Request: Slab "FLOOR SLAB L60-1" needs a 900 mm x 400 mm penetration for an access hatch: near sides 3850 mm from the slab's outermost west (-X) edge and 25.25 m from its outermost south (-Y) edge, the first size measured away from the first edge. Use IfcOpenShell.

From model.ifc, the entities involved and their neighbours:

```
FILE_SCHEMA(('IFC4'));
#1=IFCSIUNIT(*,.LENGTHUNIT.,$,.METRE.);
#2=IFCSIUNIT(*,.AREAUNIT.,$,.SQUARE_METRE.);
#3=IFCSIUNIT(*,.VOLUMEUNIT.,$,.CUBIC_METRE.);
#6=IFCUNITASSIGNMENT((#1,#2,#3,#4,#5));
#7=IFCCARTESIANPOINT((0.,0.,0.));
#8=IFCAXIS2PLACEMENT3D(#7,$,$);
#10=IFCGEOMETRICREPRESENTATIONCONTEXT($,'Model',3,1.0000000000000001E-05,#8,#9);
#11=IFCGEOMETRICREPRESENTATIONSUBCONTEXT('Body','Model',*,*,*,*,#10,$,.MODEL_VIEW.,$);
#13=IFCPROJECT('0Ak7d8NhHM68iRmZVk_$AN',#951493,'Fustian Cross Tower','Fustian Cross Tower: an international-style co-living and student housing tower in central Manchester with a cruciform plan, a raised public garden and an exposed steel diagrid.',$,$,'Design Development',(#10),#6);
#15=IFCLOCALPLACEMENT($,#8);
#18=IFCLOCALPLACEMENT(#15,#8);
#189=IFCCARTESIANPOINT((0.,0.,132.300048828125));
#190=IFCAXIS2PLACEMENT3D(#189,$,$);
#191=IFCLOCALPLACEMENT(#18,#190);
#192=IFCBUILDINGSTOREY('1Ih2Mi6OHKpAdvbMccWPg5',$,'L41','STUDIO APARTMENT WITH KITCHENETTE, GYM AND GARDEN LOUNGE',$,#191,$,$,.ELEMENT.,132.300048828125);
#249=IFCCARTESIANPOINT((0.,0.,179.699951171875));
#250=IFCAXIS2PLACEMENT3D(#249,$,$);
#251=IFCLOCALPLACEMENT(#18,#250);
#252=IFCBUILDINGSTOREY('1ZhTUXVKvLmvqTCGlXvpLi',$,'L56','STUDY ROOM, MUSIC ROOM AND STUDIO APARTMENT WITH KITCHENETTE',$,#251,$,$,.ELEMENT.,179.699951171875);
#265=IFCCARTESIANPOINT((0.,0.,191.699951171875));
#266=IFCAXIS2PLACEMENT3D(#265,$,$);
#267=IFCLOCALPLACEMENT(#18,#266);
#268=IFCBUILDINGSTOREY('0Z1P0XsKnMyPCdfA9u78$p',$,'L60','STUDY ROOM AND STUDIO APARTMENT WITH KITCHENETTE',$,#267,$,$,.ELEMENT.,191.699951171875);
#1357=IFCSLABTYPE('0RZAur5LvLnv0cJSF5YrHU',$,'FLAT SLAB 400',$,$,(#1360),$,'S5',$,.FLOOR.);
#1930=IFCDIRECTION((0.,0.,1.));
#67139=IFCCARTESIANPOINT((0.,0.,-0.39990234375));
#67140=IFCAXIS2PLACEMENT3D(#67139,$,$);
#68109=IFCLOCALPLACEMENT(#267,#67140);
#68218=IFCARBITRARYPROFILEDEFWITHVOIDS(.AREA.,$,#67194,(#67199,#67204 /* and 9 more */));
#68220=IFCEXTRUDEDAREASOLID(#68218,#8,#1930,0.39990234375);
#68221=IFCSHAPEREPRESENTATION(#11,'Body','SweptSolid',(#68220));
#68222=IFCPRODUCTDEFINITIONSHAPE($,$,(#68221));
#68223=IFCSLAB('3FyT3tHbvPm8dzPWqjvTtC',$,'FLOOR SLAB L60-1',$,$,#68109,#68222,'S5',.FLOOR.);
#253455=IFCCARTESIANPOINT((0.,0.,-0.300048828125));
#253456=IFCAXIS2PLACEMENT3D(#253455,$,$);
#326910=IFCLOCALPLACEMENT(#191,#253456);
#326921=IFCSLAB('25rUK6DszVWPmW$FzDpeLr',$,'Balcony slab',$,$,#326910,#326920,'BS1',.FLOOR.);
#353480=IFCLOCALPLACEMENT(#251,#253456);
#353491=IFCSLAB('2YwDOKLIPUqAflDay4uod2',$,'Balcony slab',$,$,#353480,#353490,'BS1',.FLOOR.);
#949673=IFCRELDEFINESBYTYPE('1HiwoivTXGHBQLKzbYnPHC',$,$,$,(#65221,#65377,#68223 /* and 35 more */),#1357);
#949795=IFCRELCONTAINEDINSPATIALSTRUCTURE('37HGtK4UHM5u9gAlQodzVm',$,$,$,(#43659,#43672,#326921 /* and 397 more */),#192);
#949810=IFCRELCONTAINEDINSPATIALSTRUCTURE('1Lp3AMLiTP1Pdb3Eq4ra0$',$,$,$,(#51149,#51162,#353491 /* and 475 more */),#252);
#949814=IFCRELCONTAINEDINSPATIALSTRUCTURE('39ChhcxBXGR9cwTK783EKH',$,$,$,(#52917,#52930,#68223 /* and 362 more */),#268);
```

```python
import numpy as np
import ifcopenshell
import ifcopenshell.api.feature
import ifcopenshell.api.geometry
import ifcopenshell.api.root
import ifcopenshell.geom
import ifcopenshell.util.placement
import ifcopenshell.util.representation
import ifcopenshell.util.shape
import ifcopenshell.util.unit

model = ifcopenshell.open("model.ifc")
unit_scale = ifcopenshell.util.unit.calculate_unit_scale(model)
settings = ifcopenshell.geom.settings()


def volume(element):
    """Net volume in cubic metres, openings subtracted."""
    shape = ifcopenshell.geom.create_shape(settings, element)
    return ifcopenshell.util.shape.get_volume(shape.geometry)


slab = model.by_id(68223)
before = volume(slab)

# Extent in the slab's own axes, in metres. The edges named are its -X and -Y sides.
slab_shape = ifcopenshell.geom.create_shape(settings, slab)
vertices = ifcopenshell.util.shape.get_vertices(slab_shape.geometry)
x_min, y_min, bottom = vertices.min(axis=0)
top = vertices[:, 2].max()

opening = ifcopenshell.api.root.create_entity(model, ifc_class="IfcOpeningElement", name="Access hatch opening", predefined_type="OPENING")
context = ifcopenshell.util.representation.get_context(model, "Model", "Body", "MODEL_VIEW")
width, depth = 0.9, 0.4
outline = [(0.0, 0.0), (width, 0.0), (width, depth), (0.0, depth), (0.0, 0.0)]
# Overshoot both faces by 50 mm so the cut is clean.
shape = ifcopenshell.api.geometry.add_slab_representation(
    model, context=context, depth=top - bottom + 0.1, polyline=outline
)
ifcopenshell.api.geometry.assign_representation(model, product=opening, representation=shape)

matrix = ifcopenshell.util.placement.get_local_placement(slab.ObjectPlacement)
matrix[:, 3] = matrix @ np.append(np.array([x_min + 3.85, y_min + 25.25, bottom - 0.05]) / unit_scale, 1.0)
ifcopenshell.api.geometry.edit_object_placement(model, product=opening, matrix=matrix, is_si=False)
ifcopenshell.api.feature.add_feature(model, feature=opening, element=slab)

after = volume(slab)

print(f"slab volume {before:.3f} -> {after:.3f} m3")

model.write("model_edited.ifc")
```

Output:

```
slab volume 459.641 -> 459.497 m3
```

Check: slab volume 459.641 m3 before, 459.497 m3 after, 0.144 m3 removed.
